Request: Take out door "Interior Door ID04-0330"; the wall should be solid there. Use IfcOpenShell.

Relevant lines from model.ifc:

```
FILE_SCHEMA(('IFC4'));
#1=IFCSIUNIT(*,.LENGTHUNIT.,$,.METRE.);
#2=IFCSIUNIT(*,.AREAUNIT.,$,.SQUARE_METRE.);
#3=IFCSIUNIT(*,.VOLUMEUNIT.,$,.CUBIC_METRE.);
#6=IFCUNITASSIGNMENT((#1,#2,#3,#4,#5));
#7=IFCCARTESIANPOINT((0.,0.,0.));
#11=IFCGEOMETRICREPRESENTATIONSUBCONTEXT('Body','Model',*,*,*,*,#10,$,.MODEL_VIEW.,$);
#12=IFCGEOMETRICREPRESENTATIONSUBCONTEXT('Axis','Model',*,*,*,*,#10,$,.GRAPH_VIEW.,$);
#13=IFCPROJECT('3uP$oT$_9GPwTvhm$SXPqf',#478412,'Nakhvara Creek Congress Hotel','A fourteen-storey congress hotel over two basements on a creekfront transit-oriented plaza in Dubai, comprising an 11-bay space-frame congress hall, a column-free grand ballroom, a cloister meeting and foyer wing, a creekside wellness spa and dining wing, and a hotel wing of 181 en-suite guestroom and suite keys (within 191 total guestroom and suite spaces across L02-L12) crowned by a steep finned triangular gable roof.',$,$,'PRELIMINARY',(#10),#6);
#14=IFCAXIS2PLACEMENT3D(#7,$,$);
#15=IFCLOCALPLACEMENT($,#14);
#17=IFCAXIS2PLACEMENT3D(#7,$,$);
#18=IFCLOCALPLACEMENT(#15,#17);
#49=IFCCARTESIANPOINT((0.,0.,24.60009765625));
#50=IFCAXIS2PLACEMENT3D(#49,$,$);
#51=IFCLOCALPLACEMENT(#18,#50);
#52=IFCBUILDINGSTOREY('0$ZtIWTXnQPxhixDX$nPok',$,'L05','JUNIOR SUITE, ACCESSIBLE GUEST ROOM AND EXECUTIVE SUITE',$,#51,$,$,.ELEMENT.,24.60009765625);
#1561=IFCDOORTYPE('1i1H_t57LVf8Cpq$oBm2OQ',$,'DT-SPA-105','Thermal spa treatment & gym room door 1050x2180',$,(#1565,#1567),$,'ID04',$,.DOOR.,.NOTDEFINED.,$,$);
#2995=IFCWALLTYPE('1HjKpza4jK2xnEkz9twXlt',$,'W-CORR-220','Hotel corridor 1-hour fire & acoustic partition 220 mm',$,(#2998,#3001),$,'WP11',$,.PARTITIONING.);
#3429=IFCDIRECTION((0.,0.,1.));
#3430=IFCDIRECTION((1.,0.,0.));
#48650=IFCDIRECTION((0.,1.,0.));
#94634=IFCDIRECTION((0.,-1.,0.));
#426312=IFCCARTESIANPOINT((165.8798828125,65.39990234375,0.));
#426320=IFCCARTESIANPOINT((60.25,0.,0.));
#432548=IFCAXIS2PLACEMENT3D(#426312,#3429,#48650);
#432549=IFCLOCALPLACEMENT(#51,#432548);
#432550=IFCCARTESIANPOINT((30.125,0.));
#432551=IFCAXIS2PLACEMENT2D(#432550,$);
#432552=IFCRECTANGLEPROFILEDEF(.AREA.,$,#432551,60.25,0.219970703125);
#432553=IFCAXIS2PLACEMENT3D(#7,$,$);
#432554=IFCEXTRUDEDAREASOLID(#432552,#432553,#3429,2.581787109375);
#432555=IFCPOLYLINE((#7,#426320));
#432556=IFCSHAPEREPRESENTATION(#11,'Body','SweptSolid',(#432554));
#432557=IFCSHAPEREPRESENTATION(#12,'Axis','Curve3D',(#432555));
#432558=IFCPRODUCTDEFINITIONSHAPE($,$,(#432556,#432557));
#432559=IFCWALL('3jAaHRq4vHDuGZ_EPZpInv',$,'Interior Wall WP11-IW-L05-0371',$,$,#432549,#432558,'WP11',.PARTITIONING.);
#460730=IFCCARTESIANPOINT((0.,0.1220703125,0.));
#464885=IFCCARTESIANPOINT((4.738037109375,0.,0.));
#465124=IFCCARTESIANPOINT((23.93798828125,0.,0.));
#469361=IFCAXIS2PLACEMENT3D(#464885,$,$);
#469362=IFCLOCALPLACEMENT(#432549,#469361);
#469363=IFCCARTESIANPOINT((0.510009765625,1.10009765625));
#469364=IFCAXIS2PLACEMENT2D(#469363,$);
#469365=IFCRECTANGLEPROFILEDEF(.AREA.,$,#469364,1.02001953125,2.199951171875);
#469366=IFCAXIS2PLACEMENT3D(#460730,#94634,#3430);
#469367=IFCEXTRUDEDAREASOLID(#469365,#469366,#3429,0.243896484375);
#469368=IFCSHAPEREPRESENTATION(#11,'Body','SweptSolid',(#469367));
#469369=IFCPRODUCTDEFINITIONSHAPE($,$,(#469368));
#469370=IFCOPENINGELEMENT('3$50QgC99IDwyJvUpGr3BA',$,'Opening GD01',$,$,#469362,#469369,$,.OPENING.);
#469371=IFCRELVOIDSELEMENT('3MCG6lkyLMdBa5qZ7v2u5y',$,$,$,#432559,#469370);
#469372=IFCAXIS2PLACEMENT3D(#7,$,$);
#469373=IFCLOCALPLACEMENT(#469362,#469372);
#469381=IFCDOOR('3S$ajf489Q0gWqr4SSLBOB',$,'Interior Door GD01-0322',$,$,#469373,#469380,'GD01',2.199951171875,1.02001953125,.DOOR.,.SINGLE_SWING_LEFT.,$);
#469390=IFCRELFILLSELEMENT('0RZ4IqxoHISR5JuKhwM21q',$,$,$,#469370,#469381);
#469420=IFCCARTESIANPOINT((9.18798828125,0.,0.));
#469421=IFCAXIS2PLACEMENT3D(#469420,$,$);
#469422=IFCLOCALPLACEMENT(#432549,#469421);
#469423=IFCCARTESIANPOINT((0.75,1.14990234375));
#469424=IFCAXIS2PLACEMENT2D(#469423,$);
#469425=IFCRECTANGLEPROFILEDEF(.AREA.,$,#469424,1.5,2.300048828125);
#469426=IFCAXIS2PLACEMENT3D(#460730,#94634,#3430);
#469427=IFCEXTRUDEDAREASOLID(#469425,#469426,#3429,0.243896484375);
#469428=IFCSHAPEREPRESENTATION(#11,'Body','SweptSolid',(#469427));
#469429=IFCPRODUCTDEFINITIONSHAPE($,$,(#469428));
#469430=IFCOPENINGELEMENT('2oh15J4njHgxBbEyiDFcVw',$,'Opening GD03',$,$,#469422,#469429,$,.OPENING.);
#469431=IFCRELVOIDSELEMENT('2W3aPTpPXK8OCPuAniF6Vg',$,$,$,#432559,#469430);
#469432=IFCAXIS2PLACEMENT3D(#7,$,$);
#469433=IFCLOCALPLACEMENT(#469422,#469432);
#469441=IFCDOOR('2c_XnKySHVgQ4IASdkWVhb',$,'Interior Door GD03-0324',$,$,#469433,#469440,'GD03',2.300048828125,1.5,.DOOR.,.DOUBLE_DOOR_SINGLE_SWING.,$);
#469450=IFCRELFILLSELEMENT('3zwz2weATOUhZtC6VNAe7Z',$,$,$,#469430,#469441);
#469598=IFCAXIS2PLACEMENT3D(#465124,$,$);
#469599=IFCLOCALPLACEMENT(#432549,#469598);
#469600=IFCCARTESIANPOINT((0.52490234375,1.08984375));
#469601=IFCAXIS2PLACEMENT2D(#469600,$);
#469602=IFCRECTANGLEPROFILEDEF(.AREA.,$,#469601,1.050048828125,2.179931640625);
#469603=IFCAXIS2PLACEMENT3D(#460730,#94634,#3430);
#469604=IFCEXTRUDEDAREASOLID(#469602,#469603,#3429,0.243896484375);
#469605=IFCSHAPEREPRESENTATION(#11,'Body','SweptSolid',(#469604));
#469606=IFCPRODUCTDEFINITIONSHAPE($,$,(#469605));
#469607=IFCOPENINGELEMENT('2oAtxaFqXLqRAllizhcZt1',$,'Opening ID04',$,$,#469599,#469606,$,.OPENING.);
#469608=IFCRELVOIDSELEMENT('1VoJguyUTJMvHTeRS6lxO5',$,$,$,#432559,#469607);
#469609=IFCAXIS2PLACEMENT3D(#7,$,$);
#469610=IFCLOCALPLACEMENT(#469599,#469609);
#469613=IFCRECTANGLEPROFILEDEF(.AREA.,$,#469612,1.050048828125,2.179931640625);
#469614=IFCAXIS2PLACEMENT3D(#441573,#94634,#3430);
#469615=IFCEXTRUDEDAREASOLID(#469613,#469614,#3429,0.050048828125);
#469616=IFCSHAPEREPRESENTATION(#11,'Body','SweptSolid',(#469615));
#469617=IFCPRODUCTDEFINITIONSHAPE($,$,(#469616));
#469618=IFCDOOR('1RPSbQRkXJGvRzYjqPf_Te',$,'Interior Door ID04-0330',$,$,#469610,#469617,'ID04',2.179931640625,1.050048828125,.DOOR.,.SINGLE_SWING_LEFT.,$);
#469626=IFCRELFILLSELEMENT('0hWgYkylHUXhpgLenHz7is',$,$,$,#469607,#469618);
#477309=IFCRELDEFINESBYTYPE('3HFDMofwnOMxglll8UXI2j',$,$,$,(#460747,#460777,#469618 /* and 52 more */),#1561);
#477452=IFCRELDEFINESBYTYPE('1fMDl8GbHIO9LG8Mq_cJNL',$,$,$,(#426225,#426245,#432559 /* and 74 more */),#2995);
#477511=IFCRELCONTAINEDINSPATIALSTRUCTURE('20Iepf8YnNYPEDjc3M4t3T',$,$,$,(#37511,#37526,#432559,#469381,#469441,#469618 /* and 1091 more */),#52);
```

```python
import ifcopenshell
import ifcopenshell.api.feature
import ifcopenshell.api.root
import ifcopenshell.geom
import ifcopenshell.util.shape

model = ifcopenshell.open("model.ifc")
settings = ifcopenshell.geom.settings()


def volume(element):
    """Net volume in cubic metres, openings subtracted."""
    shape = ifcopenshell.geom.create_shape(settings, element)
    return ifcopenshell.util.shape.get_volume(shape.geometry)


door = model.by_id(469618)
opening = door.FillsVoids[0].RelatingOpeningElement
wall = opening.VoidsElements[0].RelatingBuildingElement
before = volume(wall)

ifcopenshell.api.root.remove_product(model, product=door)
ifcopenshell.api.feature.remove_feature(model, feature=opening)

after = volume(wall)

print(f"wall volume {before:.3f} -> {after:.3f} m3")

model.write("model_rev.ifc")
```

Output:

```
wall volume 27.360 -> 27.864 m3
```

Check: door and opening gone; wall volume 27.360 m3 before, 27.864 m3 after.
